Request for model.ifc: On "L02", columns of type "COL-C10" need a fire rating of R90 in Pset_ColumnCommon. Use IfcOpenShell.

First a look at what the model holds.

```python
import ifcopenshell
import ifcopenshell.util.element

model = ifcopenshell.open("model.ifc")
print(model.schema)
storey = next(s for s in model.by_type("IfcBuildingStorey") if s.Name == "L02")
columns = [e for e in ifcopenshell.util.element.get_decomposition(storey) if e.is_a("IfcColumn")]
seen = {}
for e in columns:
    element_type = ifcopenshell.util.element.get_type(e)
    key = (element_type.Name if element_type != e and element_type else None, ifcopenshell.util.element.get_pset(e, "Pset_ColumnCommon", "FireRating"))
    seen[key] = seen.get(key, 0) + 1
for (name, value), count in sorted(seen.items(), key=str):
    print(count, "x", name, "|", value)
```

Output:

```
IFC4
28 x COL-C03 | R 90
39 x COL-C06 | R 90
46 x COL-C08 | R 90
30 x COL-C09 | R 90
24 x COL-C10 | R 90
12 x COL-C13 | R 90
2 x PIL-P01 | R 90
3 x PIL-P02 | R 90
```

```python
import ifcopenshell
import ifcopenshell.api.pset
import ifcopenshell.util.element

model = ifcopenshell.open("model.ifc")

storey = next(s for s in model.by_type("IfcBuildingStorey") if s.Name == "L02")
columns = [e for e in ifcopenshell.util.element.get_decomposition(storey) if e.is_a("IfcColumn")]

count = 0
for e in columns:
    element_type = ifcopenshell.util.element.get_type(e)
    if element_type in (None, e) or element_type.Name != "COL-C10":
        continue
    # add_pset returns the element's existing set when there is one.
    pset = ifcopenshell.api.pset.add_pset(model, product=e, name="Pset_ColumnCommon")
    ifcopenshell.api.pset.edit_pset(model, pset=pset, properties={"FireRating": "R90"})
    count += 1

print(count, "columns updated")

model.write("model_edited.ifc")
```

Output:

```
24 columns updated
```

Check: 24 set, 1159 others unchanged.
